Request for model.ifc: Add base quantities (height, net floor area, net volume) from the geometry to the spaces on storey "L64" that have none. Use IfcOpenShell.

First a look at what the model holds.

```python
import ifcopenshell
import ifcopenshell.util.element
import ifcopenshell.util.unit

model = ifcopenshell.open("model.ifc")
print(model.schema)
for unit_type in ("LENGTHUNIT", "AREAUNIT", "VOLUMEUNIT"):
    print(unit_type, ifcopenshell.util.unit.calculate_unit_scale(model, unit_type))
storey = next(s for s in model.by_type("IfcBuildingStorey") if s.Name == "L64")
spaces = [e for e in ifcopenshell.util.element.get_decomposition(storey) if e.is_a("IfcSpace")]
for e in sorted(spaces, key=lambda e: e.id()):
    print(e.id(), e.is_a(), e.Name, list(ifcopenshell.util.element.get_psets(e, qtos_only=True)), sep=" | ")
```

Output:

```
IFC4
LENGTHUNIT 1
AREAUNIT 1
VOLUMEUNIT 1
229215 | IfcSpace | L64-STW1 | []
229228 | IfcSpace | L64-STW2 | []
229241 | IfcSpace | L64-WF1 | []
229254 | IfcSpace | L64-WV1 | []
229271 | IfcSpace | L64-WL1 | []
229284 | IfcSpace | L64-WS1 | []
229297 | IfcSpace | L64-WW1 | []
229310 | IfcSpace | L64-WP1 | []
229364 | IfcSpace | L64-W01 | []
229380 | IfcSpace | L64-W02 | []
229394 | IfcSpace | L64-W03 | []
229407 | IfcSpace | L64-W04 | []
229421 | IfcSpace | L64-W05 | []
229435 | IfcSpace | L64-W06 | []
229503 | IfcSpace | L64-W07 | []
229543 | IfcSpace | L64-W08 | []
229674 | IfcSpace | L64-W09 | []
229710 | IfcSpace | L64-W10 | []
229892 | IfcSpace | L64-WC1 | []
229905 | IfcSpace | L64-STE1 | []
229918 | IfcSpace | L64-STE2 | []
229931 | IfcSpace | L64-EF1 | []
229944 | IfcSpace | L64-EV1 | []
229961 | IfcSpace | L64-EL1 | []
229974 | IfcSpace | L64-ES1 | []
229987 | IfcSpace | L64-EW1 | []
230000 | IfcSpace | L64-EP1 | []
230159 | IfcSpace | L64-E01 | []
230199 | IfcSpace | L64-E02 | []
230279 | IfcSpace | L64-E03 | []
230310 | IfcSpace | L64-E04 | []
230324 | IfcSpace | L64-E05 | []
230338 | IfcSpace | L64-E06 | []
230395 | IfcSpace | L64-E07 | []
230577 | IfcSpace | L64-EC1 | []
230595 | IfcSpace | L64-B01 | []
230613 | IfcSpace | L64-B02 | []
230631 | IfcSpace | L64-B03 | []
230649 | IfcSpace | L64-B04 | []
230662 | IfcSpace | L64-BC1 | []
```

```python
import ifcopenshell
import ifcopenshell.api.pset
import ifcopenshell.geom
import ifcopenshell.util.element
import ifcopenshell.util.shape
import ifcopenshell.util.unit

model = ifcopenshell.open("model.ifc")
unit_scale = ifcopenshell.util.unit.calculate_unit_scale(model)
area_scale = ifcopenshell.util.unit.calculate_unit_scale(model, "AREAUNIT")
volume_scale = ifcopenshell.util.unit.calculate_unit_scale(model, "VOLUMEUNIT")
settings = ifcopenshell.geom.settings()

storey = next(s for s in model.by_type("IfcBuildingStorey") if s.Name == "L64")
spaces = [e for e in ifcopenshell.util.element.get_decomposition(storey) if e.is_a("IfcSpace")]

for e in sorted(spaces, key=lambda e: e.id()):
    if ifcopenshell.util.element.get_psets(e, qtos_only=True, should_inherit=False):
        continue
    # Geometry comes back in metres, in the element's own axes.
    shape = ifcopenshell.geom.create_shape(settings, e)
    values = {
        "Height": ifcopenshell.util.shape.get_z(shape.geometry) / unit_scale,
        "NetFloorArea": ifcopenshell.util.shape.get_footprint_area(shape.geometry) / area_scale,
        "NetVolume": ifcopenshell.util.shape.get_volume(shape.geometry) / volume_scale,
    }
    qto = ifcopenshell.api.pset.add_qto(model, product=e, name="Qto_SpaceBaseQuantities")
    ifcopenshell.api.pset.edit_qto(model, qto=qto, properties=values)
    print(e.id(), {k: round(v, 3) for k, v in values.items()})

model.write("model_v2.ifc")
```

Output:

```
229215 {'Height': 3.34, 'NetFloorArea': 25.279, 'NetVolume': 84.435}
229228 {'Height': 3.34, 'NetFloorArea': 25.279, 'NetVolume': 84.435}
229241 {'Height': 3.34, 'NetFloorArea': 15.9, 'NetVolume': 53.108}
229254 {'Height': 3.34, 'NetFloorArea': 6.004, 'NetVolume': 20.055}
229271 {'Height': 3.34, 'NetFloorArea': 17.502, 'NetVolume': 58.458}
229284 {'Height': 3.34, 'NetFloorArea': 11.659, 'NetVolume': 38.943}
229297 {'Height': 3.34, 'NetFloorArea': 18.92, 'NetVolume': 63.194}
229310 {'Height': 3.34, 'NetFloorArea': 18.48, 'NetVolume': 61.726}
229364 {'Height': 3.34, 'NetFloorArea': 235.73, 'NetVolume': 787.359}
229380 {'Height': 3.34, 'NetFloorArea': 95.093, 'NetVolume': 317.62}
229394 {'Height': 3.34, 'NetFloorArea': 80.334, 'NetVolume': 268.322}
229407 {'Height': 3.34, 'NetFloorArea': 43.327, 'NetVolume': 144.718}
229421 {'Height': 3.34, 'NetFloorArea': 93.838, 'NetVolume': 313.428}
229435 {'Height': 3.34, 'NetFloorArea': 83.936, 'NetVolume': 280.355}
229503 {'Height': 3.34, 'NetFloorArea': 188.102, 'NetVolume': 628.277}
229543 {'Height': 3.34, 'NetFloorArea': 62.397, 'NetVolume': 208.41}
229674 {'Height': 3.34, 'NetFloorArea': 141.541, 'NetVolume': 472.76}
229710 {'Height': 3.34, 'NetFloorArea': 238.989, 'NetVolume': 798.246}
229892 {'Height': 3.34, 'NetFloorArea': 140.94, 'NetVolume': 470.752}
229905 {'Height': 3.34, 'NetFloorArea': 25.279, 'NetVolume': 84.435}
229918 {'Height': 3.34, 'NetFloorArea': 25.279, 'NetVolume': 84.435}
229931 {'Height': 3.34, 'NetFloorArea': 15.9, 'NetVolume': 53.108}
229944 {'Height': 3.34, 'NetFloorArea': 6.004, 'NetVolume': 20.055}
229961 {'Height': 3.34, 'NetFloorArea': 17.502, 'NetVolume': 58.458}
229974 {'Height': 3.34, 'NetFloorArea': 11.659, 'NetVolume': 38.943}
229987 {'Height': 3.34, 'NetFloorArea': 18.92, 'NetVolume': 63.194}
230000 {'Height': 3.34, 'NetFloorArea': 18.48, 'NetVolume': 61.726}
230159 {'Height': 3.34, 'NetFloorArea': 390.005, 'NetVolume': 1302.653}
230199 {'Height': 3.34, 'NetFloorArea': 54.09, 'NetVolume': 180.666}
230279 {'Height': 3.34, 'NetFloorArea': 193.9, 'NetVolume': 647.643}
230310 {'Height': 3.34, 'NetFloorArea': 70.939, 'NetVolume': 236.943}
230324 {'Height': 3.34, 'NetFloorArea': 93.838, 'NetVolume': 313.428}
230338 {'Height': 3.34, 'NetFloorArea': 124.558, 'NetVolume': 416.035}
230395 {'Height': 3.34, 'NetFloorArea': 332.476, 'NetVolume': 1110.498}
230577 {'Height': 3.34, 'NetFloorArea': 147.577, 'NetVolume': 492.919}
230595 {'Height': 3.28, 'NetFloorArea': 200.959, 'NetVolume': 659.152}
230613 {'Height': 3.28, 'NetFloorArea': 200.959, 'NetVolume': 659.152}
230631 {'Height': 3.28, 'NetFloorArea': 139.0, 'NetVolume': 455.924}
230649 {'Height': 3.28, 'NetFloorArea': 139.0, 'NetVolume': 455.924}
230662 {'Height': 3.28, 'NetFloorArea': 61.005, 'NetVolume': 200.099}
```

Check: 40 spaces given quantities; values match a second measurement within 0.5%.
